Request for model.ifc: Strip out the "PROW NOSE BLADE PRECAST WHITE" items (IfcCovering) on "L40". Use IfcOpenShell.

First a look at what the model holds.

```python
import ifcopenshell
import ifcopenshell.util.element

model = ifcopenshell.open("model.ifc")
print(model.schema)
storey = next(s for s in model.by_type("IfcBuildingStorey") if s.Name == "L40")
coverings = [e for e in ifcopenshell.util.element.get_decomposition(storey) if e.is_a("IfcCovering")]
seen = {}
for e in coverings:
    element_type = ifcopenshell.util.element.get_type(e)
    name = element_type.Name if element_type not in (None, e) else None
    seen[name] = seen.get(name, 0) + 1
for name, count in sorted(seen.items(), key=str):
    print(count, "x", name)
```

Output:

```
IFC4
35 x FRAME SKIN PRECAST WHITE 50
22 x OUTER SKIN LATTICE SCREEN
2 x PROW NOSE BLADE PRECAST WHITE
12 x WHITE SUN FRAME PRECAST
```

```python
import ifcopenshell
import ifcopenshell.api.root
import ifcopenshell.util.element

model = ifcopenshell.open("model.ifc")

storey = next(s for s in model.by_type("IfcBuildingStorey") if s.Name == "L40")
coverings = [e for e in ifcopenshell.util.element.get_decomposition(storey) if e.is_a("IfcCovering")]
targets = [e for e in coverings if (t := ifcopenshell.util.element.get_type(e)) not in (None, e) and t.Name == "PROW NOSE BLADE PRECAST WHITE"]

for e in targets:
    ifcopenshell.api.root.remove_product(model, product=e)
print(len(targets), "removed")

model.write("model_rev.ifc")
```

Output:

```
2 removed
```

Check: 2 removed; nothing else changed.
